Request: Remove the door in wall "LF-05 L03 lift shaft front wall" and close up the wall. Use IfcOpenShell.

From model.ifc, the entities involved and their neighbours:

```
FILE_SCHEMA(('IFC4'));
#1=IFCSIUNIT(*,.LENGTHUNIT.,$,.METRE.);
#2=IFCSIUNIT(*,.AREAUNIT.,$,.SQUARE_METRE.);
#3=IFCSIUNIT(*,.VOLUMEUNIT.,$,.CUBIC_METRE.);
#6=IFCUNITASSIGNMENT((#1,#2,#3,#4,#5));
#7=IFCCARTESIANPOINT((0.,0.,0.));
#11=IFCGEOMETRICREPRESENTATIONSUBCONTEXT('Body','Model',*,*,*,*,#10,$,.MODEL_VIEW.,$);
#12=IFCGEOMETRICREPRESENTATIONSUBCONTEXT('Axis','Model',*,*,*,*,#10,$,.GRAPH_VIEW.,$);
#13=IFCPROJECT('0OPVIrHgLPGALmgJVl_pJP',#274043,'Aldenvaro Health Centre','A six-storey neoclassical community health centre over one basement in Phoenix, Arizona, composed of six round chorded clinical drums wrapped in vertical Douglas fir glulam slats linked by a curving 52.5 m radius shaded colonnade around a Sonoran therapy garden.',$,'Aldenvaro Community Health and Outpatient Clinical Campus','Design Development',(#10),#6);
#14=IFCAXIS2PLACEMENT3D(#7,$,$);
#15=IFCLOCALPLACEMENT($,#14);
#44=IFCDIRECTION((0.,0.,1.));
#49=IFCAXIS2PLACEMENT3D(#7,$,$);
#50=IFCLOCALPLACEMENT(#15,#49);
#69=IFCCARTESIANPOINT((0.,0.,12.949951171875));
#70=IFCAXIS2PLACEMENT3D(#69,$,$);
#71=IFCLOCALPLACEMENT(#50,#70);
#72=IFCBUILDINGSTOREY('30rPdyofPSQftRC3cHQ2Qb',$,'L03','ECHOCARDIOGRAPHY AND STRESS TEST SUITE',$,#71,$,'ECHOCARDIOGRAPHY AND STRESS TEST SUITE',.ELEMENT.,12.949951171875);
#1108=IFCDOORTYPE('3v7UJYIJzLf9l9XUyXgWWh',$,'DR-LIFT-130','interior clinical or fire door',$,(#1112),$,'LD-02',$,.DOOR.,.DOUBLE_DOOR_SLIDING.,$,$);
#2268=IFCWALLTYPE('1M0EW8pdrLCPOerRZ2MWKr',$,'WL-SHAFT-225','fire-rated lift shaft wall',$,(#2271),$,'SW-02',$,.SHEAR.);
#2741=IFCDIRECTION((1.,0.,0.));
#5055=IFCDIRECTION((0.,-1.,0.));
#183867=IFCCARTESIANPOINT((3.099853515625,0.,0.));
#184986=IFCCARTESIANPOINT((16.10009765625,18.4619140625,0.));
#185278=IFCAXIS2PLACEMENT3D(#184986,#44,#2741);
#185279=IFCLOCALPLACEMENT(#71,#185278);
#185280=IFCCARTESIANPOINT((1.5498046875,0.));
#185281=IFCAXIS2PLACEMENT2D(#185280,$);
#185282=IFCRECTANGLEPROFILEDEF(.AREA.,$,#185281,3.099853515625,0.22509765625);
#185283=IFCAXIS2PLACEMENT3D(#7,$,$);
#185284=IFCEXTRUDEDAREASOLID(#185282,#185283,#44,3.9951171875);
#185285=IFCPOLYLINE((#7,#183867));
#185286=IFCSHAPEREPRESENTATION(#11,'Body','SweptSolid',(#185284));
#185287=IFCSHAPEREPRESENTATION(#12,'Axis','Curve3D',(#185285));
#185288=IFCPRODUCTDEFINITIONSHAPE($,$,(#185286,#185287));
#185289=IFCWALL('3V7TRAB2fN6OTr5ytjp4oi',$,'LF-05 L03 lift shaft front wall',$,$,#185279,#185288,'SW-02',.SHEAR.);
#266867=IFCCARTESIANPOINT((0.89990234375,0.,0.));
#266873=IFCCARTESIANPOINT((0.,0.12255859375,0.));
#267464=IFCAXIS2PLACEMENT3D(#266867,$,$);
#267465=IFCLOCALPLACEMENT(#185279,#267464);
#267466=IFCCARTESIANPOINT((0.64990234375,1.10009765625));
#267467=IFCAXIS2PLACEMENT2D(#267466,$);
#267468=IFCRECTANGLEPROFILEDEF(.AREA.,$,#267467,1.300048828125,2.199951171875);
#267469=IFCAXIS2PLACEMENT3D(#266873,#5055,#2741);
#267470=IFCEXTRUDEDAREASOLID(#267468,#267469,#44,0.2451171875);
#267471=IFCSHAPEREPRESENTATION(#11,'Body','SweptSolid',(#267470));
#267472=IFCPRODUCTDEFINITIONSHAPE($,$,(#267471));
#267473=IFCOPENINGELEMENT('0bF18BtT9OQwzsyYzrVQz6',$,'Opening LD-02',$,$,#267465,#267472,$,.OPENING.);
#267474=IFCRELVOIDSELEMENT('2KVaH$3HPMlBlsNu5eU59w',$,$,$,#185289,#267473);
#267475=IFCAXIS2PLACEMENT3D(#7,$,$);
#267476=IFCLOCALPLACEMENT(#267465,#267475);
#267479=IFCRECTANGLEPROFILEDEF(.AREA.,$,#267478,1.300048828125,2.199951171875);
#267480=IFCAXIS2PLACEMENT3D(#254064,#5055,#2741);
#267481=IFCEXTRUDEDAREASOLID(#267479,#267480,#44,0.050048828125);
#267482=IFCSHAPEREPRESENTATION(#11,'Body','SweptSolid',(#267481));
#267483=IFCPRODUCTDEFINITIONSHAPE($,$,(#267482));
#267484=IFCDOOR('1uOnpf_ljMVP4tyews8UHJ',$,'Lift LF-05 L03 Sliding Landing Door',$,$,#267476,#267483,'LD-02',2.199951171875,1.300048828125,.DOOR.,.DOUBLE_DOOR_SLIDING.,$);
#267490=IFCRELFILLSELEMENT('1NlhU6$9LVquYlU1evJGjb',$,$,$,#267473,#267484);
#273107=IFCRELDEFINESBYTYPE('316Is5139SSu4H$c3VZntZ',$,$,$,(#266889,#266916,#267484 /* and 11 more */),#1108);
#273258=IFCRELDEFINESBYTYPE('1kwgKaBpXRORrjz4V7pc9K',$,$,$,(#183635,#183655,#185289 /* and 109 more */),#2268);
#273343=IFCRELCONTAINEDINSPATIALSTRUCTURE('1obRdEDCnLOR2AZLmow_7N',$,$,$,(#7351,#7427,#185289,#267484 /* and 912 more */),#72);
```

```python
import ifcopenshell
import ifcopenshell.api.feature
import ifcopenshell.api.root
import ifcopenshell.geom
import ifcopenshell.util.shape

model = ifcopenshell.open("model.ifc")
settings = ifcopenshell.geom.settings()


def volume(element):
    """Net volume in cubic metres, openings subtracted."""
    shape = ifcopenshell.geom.create_shape(settings, element)
    return ifcopenshell.util.shape.get_volume(shape.geometry)


door = model.by_id(267484)
opening = door.FillsVoids[0].RelatingOpeningElement
wall = opening.VoidsElements[0].RelatingBuildingElement
before = volume(wall)

ifcopenshell.api.root.remove_product(model, product=door)
ifcopenshell.api.feature.remove_feature(model, feature=opening)

after = volume(wall)

print(f"wall volume {before:.3f} -> {after:.3f} m3")

model.write("model_rev.ifc")
```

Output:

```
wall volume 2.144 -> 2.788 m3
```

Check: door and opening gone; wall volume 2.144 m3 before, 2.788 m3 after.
